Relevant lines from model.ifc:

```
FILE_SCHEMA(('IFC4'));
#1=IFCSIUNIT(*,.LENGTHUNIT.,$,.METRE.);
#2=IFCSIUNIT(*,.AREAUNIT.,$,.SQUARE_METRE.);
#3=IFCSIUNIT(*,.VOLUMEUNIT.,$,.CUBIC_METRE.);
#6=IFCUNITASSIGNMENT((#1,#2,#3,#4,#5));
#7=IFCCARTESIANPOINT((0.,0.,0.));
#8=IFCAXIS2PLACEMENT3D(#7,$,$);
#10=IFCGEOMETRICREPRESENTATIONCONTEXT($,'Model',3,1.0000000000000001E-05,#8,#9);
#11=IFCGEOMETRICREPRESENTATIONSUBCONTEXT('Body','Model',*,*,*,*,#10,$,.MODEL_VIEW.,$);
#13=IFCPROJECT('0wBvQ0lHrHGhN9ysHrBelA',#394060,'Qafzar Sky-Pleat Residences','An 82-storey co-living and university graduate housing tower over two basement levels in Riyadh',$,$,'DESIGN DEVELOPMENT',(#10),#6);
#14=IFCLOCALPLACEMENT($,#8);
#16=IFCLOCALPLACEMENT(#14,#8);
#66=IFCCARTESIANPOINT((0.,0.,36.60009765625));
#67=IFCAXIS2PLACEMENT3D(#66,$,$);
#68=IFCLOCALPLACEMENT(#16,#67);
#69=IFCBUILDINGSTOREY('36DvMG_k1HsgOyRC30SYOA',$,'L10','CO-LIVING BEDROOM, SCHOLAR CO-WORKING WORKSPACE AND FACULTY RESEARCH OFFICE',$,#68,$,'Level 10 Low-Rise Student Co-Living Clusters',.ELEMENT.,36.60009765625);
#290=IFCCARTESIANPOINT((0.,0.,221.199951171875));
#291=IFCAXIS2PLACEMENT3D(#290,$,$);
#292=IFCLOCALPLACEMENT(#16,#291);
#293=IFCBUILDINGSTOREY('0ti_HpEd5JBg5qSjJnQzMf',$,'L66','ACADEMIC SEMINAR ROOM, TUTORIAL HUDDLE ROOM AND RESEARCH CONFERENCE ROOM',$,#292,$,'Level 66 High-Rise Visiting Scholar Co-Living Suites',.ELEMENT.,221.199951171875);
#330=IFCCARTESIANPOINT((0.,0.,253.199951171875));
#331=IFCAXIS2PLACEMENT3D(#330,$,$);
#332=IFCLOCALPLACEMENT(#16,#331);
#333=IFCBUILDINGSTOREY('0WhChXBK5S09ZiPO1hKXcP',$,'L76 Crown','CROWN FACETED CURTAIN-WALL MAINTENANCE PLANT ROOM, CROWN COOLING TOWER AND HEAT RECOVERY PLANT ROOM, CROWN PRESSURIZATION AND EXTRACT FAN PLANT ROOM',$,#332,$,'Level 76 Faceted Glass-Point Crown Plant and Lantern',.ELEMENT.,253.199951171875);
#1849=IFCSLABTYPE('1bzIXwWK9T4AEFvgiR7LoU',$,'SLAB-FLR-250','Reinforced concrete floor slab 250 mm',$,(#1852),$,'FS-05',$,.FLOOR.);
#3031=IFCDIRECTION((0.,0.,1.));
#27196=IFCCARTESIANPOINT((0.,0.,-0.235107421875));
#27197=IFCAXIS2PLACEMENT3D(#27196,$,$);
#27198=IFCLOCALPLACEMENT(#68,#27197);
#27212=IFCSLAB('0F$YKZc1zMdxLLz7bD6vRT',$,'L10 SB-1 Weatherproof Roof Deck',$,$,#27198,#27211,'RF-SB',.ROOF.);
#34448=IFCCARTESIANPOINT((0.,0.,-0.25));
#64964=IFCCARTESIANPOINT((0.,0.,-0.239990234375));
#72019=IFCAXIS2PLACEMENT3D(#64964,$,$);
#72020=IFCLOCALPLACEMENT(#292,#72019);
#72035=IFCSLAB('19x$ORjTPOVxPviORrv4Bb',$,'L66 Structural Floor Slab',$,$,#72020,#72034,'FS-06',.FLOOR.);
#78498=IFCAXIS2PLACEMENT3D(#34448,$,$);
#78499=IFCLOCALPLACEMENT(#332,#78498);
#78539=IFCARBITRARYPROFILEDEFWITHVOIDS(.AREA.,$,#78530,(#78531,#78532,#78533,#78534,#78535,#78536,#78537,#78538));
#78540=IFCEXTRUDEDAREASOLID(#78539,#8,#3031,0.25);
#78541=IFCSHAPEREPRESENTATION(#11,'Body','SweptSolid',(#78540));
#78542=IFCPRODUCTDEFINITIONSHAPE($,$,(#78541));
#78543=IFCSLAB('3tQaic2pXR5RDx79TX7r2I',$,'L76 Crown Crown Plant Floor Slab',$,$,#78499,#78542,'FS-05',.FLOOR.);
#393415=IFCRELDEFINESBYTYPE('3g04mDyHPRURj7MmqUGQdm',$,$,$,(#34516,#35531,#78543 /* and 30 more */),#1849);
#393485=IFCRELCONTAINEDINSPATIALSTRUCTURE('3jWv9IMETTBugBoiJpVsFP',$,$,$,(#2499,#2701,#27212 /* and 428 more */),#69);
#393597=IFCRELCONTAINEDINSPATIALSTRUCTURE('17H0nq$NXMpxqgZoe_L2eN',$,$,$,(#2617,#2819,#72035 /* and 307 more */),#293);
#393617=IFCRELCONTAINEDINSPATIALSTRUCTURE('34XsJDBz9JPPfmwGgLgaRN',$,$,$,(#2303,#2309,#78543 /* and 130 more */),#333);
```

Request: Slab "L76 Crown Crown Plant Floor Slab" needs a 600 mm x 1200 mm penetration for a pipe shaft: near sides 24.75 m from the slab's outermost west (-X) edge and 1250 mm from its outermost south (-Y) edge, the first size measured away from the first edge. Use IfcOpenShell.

```python
import numpy as np
import ifcopenshell
import ifcopenshell.api.feature
import ifcopenshell.api.geometry
import ifcopenshell.api.root
import ifcopenshell.geom
import ifcopenshell.util.placement
import ifcopenshell.util.representation
import ifcopenshell.util.shape
import ifcopenshell.util.unit

model = ifcopenshell.open("model.ifc")
unit_scale = ifcopenshell.util.unit.calculate_unit_scale(model)
settings = ifcopenshell.geom.settings()


def volume(element):
    """Net volume in cubic metres, openings subtracted."""
    shape = ifcopenshell.geom.create_shape(settings, element)
    return ifcopenshell.util.shape.get_volume(shape.geometry)


slab = model.by_guid("3tQaic2pXR5RDx79TX7r2I")
before = volume(slab)

# Extent in the slab's own axes, in metres. The edges named are its -X and -Y sides.
slab_shape = ifcopenshell.geom.create_shape(settings, slab)
vertices = ifcopenshell.util.shape.get_vertices(slab_shape.geometry)
x_min, y_min, bottom = vertices.min(axis=0)
top = vertices[:, 2].max()

opening = ifcopenshell.api.root.create_entity(model, ifc_class="IfcOpeningElement", name="Pipe shaft opening", predefined_type="OPENING")
context = ifcopenshell.util.representation.get_context(model, "Model", "Body", "MODEL_VIEW")
width, depth = 0.6, 1.2
outline = [(0.0, 0.0), (width, 0.0), (width, depth), (0.0, depth), (0.0, 0.0)]
# Overshoot both faces by 50 mm so the cut is clean.
shape = ifcopenshell.api.geometry.add_slab_representation(
    model, context=context, depth=top - bottom + 0.1, polyline=outline
)
ifcopenshell.api.geometry.assign_representation(model, product=opening, representation=shape)

matrix = ifcopenshell.util.placement.get_local_placement(slab.ObjectPlacement)
matrix[:, 3] = matrix @ np.append(np.array([x_min + 24.75, y_min + 1.25, bottom - 0.05]) / unit_scale, 1.0)
ifcopenshell.api.geometry.edit_object_placement(model, product=opening, matrix=matrix, is_si=False)
ifcopenshell.api.feature.add_feature(model, feature=opening, element=slab)

after = volume(slab)

print(f"slab volume {before:.3f} -> {after:.3f} m3")

model.write("model-out.ifc")
```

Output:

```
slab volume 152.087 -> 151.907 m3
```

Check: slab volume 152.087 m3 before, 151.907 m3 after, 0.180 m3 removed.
